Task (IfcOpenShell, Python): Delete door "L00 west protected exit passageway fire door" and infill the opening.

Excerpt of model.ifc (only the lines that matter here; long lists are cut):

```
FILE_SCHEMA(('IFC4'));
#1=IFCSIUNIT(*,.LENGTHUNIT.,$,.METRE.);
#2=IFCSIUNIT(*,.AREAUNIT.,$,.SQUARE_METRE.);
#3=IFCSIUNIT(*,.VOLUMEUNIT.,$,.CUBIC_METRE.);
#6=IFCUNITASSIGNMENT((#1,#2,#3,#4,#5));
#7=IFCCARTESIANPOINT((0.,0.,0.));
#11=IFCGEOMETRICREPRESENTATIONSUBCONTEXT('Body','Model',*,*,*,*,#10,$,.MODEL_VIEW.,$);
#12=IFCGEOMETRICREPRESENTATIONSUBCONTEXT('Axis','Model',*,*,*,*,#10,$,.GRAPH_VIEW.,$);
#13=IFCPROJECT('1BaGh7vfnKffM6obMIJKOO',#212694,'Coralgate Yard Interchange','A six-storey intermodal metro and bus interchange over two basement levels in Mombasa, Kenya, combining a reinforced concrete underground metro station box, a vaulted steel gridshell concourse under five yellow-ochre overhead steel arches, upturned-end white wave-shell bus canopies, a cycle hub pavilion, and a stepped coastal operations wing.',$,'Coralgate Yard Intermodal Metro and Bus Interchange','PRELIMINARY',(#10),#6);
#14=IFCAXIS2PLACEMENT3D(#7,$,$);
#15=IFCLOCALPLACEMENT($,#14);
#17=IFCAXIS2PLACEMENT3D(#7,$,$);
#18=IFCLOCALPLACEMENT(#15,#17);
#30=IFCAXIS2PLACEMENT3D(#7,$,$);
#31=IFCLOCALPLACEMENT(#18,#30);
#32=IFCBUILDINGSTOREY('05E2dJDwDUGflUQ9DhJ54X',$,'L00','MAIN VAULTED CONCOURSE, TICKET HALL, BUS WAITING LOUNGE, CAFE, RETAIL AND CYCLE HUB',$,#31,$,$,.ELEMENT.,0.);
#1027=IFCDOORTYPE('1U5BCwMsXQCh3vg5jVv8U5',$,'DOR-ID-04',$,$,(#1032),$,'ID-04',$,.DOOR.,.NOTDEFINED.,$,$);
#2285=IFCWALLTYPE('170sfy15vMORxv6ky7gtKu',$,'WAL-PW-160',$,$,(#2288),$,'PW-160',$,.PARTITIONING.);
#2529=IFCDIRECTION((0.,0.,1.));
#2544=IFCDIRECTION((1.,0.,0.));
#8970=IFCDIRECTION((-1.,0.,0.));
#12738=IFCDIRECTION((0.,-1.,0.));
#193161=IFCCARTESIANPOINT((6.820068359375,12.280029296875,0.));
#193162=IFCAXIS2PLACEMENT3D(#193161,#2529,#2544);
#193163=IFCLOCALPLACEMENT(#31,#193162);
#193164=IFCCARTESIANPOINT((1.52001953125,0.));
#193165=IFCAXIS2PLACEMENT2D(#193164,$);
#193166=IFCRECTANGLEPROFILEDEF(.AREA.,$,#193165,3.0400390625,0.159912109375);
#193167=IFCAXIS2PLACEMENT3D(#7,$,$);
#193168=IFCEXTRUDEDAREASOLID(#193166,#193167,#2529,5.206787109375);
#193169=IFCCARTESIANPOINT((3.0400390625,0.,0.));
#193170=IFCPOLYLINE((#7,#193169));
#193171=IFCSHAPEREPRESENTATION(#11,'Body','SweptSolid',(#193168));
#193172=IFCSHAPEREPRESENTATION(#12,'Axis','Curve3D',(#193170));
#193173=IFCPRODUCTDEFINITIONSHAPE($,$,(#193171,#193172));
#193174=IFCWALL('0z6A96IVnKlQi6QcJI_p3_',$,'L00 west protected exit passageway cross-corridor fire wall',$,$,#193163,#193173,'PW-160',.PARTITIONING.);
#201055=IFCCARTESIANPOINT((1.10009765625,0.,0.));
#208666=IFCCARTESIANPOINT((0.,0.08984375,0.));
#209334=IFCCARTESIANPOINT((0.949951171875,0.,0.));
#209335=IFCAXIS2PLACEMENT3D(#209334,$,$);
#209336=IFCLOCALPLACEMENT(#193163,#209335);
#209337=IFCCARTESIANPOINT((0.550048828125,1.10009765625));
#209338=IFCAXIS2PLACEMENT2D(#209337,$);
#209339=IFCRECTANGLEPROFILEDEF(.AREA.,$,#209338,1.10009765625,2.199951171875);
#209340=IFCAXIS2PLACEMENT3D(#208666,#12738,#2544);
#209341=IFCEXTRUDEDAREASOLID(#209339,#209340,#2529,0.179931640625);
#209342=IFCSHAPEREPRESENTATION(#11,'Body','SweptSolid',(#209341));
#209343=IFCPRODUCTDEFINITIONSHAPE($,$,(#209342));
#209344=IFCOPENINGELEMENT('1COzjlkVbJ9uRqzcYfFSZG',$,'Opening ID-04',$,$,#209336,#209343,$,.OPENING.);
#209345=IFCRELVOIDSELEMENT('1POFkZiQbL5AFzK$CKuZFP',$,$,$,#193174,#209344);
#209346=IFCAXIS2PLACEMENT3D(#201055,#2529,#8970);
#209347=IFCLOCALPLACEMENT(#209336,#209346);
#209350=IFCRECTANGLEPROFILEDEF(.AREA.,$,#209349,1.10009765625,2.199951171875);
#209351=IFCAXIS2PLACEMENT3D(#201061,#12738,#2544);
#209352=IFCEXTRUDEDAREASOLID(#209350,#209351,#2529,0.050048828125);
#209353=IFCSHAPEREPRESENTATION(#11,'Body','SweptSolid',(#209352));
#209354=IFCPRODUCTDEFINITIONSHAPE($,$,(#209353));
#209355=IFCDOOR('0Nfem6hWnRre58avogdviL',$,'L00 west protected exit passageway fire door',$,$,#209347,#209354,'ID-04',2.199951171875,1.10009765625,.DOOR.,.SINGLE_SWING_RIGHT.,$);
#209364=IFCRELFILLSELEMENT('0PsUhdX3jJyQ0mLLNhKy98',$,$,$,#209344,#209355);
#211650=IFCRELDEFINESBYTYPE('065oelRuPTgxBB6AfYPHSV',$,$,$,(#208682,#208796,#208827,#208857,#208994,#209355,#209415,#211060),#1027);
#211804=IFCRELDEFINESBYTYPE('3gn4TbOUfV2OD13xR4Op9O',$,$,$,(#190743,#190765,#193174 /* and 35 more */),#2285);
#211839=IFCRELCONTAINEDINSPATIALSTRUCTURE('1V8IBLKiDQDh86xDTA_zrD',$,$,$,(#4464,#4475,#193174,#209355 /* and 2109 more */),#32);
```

```python
import ifcopenshell
import ifcopenshell.api.feature
import ifcopenshell.api.root
import ifcopenshell.geom
import ifcopenshell.util.shape

model = ifcopenshell.open("model.ifc")
settings = ifcopenshell.geom.settings()


def volume(element):
    """Net volume in cubic metres, openings subtracted."""
    shape = ifcopenshell.geom.create_shape(settings, element)
    return ifcopenshell.util.shape.get_volume(shape.geometry)


door = model.by_guid("0Nfem6hWnRre58avogdviL")
opening = door.FillsVoids[0].RelatingOpeningElement
wall = opening.VoidsElements[0].RelatingBuildingElement
before = volume(wall)

ifcopenshell.api.root.remove_product(model, product=door)
ifcopenshell.api.feature.remove_feature(model, feature=opening)

after = volume(wall)

print(f"wall volume {before:.3f} -> {after:.3f} m3")

model.write("model_edited.ifc")
```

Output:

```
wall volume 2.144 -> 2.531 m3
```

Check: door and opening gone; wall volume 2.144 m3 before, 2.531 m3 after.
